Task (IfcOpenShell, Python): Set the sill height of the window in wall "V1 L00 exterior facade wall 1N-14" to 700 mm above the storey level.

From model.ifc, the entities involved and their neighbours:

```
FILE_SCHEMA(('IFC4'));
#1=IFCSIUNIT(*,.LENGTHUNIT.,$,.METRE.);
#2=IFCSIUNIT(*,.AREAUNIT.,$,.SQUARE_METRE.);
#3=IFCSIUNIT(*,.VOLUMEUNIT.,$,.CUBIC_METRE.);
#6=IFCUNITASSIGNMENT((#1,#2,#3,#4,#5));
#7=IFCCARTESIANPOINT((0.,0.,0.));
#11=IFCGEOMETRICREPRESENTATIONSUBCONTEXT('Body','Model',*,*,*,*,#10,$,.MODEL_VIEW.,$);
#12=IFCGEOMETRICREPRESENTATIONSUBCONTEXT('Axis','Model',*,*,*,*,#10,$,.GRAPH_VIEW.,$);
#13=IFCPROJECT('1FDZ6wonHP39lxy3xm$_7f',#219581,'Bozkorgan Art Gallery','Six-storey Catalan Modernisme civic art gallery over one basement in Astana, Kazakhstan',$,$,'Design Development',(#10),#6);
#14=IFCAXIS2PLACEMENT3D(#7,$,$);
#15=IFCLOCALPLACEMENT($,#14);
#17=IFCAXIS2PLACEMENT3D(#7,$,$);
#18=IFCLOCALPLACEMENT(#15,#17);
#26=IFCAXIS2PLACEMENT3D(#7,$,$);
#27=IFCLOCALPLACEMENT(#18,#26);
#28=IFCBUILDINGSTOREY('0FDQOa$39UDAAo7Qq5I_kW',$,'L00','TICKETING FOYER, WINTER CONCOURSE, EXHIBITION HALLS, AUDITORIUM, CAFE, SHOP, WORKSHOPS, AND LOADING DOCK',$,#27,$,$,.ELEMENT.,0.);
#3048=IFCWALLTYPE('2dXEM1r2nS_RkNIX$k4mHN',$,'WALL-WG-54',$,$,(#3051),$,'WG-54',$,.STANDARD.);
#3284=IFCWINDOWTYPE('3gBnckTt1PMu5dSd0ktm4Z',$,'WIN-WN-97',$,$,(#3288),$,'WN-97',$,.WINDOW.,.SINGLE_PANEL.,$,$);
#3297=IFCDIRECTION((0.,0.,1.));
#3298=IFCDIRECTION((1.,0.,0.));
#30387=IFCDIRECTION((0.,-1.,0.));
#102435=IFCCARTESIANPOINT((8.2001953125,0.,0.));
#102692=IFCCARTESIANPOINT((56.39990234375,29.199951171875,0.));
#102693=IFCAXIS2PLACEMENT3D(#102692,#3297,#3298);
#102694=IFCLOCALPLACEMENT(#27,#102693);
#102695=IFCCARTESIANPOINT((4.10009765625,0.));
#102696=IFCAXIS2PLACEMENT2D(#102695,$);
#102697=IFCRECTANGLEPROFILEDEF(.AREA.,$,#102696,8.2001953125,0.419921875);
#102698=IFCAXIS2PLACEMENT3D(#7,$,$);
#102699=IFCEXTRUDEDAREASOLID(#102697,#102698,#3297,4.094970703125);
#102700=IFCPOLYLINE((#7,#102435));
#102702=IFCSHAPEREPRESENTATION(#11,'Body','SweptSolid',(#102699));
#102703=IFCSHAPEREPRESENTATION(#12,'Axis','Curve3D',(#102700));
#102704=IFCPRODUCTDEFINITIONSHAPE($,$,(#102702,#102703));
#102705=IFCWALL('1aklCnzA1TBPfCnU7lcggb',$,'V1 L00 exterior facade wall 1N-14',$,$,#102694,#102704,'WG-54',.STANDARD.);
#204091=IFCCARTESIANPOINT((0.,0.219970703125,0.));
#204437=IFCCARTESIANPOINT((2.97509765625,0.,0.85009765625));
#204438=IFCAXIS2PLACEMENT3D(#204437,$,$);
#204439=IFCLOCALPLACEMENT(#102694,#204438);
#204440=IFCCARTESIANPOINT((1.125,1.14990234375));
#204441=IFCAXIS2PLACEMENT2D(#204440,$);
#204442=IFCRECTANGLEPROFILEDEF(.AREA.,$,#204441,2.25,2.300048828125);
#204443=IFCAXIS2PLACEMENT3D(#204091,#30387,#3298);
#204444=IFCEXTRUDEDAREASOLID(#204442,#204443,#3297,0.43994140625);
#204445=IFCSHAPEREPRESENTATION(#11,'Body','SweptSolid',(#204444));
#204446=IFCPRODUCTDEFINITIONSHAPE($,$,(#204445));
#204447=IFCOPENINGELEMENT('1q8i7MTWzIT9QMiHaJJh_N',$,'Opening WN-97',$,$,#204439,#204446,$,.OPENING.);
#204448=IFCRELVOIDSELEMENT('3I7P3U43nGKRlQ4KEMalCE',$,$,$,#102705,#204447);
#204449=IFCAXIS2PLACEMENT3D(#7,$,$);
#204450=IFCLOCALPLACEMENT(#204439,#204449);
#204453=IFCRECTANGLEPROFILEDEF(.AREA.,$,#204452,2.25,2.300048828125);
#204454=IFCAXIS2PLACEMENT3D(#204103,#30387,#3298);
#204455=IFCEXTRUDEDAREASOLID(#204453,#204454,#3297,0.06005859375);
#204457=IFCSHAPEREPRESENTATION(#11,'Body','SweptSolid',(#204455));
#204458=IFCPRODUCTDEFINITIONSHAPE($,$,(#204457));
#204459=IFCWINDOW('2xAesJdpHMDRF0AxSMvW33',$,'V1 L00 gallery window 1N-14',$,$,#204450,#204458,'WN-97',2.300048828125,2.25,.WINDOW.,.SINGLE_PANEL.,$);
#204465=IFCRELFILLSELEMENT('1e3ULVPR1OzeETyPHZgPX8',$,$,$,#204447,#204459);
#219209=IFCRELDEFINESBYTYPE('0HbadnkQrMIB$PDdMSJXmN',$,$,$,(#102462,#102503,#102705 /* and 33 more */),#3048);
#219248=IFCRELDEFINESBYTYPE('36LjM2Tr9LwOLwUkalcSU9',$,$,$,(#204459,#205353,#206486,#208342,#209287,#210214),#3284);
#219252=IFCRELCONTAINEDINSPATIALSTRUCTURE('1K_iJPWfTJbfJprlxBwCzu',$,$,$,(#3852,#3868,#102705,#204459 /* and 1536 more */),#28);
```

```python
import numpy as np
import ifcopenshell
import ifcopenshell.api.geometry
import ifcopenshell.geom
import ifcopenshell.util.element
import ifcopenshell.util.placement
import ifcopenshell.util.shape
import ifcopenshell.util.unit

model = ifcopenshell.open("model.ifc")
unit_scale = ifcopenshell.util.unit.calculate_unit_scale(model)

window = model.by_guid("2xAesJdpHMDRF0AxSMvW33")
opening = window.FillsVoids[0].RelatingOpeningElement
storey = ifcopenshell.util.element.get_container(window, ifc_class="IfcBuildingStorey")
level = ifcopenshell.util.placement.get_local_placement(storey.ObjectPlacement)[2, 3]

# The opening's origin need not be at the sill, so measure its lowest point.
shape = ifcopenshell.geom.create_shape(ifcopenshell.geom.settings(), opening)
bottom = ifcopenshell.util.shape.get_shape_bottom_elevation(shape, shape.geometry) / unit_scale
dz = level + 0.7 / unit_scale - bottom

shift = np.array([0.0, 0.0, dz])
# The window is placed relative to its opening, so it follows when the opening moves.
matrix = ifcopenshell.util.placement.get_local_placement(opening.ObjectPlacement)
matrix[:3, 3] += shift
ifcopenshell.api.geometry.edit_object_placement(
    model, product=opening, matrix=matrix, is_si=False, should_transform_children=True
)

print(f"moved by {dz * unit_scale:+.3f} m")

model.write("model_v2.ifc")
```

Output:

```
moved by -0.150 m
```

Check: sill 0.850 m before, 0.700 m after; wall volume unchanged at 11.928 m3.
